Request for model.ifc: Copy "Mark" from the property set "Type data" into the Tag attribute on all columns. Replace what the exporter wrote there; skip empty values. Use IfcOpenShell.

First a look at what the model holds.

```python
import ifcopenshell
import ifcopenshell.util.element

model = ifcopenshell.open("model.ifc")
print(model.schema)
columns = model.by_type("IfcColumn")
print(len(columns), "columns")
for e in columns[:8]:
    source = ifcopenshell.util.element.get_pset(e, "Type data", "Mark")
    target = e.Tag
    print(e.id(), repr(source), repr(target), sep=" | ")
```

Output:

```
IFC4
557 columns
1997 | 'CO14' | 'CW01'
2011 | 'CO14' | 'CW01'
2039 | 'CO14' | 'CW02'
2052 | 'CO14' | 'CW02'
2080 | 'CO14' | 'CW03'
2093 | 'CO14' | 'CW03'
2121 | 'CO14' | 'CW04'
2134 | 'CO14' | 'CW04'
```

```python
import ifcopenshell
import ifcopenshell.util.element

model = ifcopenshell.open("model.ifc")

count = 0
for e in model.by_type("IfcColumn"):
    value = ifcopenshell.util.element.get_pset(e, "Type data", "Mark")
    current = e.Tag
    if not value or not value.strip() or current == value:
        continue
    e.Tag = value
    count += 1

print(count, "columns updated")

model.write("model-out.ifc")
```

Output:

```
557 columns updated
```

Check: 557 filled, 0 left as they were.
